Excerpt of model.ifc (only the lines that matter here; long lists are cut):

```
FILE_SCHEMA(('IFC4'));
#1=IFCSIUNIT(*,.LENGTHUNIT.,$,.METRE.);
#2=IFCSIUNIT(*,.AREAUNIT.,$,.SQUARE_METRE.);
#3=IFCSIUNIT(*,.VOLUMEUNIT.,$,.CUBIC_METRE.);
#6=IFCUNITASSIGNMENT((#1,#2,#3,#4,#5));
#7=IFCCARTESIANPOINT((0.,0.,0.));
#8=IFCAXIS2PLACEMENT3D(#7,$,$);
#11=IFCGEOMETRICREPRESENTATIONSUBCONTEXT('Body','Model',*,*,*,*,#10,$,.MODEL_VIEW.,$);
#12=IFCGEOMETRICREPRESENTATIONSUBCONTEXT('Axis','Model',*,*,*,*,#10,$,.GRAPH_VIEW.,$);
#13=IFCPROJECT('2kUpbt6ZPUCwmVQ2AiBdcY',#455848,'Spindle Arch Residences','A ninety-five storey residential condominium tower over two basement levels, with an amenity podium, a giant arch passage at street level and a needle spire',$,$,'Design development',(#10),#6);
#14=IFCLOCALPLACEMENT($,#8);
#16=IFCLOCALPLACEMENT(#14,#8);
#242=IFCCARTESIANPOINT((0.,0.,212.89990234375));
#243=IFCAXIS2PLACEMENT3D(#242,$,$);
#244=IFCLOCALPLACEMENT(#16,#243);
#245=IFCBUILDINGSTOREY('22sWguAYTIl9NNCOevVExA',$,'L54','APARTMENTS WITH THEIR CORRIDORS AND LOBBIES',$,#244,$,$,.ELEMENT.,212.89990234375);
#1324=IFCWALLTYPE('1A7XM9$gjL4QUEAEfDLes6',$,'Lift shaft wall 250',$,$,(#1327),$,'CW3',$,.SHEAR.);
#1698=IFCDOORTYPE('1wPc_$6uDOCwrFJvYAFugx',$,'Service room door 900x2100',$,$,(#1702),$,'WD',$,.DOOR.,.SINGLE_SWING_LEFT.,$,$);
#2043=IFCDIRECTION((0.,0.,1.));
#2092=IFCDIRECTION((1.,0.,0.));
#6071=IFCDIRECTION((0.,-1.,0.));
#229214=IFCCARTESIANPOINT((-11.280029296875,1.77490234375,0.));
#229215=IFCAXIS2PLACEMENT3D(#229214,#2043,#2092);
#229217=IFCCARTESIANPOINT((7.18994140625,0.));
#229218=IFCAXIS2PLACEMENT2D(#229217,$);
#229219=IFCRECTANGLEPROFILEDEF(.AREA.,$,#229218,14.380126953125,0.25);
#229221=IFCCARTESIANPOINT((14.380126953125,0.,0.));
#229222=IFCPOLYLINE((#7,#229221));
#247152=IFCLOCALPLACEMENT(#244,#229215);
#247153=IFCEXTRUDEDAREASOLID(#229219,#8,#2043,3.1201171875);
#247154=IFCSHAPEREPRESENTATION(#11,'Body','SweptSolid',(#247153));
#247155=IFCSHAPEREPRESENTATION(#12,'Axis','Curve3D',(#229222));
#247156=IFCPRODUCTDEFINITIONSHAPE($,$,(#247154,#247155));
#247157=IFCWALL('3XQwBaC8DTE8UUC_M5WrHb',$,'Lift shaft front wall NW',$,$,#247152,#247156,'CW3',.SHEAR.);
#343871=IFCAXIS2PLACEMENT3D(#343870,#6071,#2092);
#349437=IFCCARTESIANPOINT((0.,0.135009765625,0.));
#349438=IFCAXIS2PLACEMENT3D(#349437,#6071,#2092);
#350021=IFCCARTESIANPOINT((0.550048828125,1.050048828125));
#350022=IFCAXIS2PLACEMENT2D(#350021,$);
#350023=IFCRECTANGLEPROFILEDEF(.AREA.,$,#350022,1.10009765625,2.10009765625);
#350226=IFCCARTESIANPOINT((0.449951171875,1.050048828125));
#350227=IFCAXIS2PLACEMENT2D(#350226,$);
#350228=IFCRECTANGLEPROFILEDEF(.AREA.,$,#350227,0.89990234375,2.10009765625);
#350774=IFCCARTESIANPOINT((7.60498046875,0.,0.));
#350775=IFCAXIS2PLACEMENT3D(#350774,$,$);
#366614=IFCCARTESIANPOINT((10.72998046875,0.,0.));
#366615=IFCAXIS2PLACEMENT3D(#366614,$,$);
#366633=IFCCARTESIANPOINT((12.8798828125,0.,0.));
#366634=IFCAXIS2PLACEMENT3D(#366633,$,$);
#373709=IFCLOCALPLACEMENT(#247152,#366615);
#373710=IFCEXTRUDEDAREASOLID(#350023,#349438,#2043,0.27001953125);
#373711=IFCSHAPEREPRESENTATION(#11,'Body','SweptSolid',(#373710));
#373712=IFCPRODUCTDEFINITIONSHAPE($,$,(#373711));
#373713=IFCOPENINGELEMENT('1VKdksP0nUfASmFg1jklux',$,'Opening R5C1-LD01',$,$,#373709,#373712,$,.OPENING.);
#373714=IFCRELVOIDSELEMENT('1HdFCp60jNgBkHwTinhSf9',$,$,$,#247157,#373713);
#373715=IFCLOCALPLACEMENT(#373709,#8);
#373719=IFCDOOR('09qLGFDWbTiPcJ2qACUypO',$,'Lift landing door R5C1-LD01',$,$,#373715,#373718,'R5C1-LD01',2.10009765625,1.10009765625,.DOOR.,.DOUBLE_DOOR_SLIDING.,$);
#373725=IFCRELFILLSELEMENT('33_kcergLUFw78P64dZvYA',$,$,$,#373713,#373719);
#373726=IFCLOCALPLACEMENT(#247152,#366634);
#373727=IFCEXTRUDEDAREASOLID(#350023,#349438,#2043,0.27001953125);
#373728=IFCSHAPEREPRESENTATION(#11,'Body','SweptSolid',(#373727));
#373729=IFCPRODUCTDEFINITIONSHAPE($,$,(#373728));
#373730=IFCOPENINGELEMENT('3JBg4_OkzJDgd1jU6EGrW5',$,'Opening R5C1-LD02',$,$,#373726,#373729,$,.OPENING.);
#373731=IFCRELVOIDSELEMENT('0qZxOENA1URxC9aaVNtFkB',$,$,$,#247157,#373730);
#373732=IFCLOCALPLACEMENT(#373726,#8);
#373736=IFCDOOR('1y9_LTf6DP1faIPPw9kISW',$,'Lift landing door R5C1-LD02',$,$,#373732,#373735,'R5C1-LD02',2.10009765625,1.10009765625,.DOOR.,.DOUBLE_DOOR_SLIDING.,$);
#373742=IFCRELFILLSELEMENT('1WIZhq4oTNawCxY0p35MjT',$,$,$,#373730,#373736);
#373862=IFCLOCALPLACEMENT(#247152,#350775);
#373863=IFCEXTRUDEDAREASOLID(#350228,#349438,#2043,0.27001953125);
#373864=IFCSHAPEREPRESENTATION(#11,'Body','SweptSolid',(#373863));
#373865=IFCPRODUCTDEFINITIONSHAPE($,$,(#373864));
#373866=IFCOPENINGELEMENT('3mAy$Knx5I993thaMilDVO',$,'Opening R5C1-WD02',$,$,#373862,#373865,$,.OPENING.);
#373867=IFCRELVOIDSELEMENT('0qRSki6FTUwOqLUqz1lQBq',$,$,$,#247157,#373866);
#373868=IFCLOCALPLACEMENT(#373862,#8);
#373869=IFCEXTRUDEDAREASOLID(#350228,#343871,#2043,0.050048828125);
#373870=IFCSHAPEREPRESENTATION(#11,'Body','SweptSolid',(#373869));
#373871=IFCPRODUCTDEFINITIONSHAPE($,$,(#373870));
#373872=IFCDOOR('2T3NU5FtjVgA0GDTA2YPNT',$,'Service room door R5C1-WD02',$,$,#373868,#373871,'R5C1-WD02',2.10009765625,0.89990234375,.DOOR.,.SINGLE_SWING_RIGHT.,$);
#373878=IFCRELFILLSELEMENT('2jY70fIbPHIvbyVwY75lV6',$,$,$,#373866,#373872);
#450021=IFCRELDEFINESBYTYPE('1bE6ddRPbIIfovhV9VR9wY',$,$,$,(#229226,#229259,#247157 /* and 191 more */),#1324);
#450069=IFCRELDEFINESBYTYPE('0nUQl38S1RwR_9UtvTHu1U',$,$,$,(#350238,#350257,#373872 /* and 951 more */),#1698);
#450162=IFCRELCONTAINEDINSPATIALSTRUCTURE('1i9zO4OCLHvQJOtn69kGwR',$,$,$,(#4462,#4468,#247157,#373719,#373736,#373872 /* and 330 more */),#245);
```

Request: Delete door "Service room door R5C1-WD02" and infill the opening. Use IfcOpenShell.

```python
import ifcopenshell
import ifcopenshell.api.feature
import ifcopenshell.api.root
import ifcopenshell.geom
import ifcopenshell.util.shape

model = ifcopenshell.open("model.ifc")
settings = ifcopenshell.geom.settings()


def volume(element):
    """Net volume in cubic metres, openings subtracted."""
    shape = ifcopenshell.geom.create_shape(settings, element)
    return ifcopenshell.util.shape.get_volume(shape.geometry)


door = model.by_guid("2T3NU5FtjVgA0GDTA2YPNT")
opening = door.FillsVoids[0].RelatingOpeningElement
wall = opening.VoidsElements[0].RelatingBuildingElement
before = volume(wall)

ifcopenshell.api.root.remove_product(model, product=door)
ifcopenshell.api.feature.remove_feature(model, feature=opening)

after = volume(wall)

print(f"wall volume {before:.3f} -> {after:.3f} m3")

model.write("model_edited.ifc")
```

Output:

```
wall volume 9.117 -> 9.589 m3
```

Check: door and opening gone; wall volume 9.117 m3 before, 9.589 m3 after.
